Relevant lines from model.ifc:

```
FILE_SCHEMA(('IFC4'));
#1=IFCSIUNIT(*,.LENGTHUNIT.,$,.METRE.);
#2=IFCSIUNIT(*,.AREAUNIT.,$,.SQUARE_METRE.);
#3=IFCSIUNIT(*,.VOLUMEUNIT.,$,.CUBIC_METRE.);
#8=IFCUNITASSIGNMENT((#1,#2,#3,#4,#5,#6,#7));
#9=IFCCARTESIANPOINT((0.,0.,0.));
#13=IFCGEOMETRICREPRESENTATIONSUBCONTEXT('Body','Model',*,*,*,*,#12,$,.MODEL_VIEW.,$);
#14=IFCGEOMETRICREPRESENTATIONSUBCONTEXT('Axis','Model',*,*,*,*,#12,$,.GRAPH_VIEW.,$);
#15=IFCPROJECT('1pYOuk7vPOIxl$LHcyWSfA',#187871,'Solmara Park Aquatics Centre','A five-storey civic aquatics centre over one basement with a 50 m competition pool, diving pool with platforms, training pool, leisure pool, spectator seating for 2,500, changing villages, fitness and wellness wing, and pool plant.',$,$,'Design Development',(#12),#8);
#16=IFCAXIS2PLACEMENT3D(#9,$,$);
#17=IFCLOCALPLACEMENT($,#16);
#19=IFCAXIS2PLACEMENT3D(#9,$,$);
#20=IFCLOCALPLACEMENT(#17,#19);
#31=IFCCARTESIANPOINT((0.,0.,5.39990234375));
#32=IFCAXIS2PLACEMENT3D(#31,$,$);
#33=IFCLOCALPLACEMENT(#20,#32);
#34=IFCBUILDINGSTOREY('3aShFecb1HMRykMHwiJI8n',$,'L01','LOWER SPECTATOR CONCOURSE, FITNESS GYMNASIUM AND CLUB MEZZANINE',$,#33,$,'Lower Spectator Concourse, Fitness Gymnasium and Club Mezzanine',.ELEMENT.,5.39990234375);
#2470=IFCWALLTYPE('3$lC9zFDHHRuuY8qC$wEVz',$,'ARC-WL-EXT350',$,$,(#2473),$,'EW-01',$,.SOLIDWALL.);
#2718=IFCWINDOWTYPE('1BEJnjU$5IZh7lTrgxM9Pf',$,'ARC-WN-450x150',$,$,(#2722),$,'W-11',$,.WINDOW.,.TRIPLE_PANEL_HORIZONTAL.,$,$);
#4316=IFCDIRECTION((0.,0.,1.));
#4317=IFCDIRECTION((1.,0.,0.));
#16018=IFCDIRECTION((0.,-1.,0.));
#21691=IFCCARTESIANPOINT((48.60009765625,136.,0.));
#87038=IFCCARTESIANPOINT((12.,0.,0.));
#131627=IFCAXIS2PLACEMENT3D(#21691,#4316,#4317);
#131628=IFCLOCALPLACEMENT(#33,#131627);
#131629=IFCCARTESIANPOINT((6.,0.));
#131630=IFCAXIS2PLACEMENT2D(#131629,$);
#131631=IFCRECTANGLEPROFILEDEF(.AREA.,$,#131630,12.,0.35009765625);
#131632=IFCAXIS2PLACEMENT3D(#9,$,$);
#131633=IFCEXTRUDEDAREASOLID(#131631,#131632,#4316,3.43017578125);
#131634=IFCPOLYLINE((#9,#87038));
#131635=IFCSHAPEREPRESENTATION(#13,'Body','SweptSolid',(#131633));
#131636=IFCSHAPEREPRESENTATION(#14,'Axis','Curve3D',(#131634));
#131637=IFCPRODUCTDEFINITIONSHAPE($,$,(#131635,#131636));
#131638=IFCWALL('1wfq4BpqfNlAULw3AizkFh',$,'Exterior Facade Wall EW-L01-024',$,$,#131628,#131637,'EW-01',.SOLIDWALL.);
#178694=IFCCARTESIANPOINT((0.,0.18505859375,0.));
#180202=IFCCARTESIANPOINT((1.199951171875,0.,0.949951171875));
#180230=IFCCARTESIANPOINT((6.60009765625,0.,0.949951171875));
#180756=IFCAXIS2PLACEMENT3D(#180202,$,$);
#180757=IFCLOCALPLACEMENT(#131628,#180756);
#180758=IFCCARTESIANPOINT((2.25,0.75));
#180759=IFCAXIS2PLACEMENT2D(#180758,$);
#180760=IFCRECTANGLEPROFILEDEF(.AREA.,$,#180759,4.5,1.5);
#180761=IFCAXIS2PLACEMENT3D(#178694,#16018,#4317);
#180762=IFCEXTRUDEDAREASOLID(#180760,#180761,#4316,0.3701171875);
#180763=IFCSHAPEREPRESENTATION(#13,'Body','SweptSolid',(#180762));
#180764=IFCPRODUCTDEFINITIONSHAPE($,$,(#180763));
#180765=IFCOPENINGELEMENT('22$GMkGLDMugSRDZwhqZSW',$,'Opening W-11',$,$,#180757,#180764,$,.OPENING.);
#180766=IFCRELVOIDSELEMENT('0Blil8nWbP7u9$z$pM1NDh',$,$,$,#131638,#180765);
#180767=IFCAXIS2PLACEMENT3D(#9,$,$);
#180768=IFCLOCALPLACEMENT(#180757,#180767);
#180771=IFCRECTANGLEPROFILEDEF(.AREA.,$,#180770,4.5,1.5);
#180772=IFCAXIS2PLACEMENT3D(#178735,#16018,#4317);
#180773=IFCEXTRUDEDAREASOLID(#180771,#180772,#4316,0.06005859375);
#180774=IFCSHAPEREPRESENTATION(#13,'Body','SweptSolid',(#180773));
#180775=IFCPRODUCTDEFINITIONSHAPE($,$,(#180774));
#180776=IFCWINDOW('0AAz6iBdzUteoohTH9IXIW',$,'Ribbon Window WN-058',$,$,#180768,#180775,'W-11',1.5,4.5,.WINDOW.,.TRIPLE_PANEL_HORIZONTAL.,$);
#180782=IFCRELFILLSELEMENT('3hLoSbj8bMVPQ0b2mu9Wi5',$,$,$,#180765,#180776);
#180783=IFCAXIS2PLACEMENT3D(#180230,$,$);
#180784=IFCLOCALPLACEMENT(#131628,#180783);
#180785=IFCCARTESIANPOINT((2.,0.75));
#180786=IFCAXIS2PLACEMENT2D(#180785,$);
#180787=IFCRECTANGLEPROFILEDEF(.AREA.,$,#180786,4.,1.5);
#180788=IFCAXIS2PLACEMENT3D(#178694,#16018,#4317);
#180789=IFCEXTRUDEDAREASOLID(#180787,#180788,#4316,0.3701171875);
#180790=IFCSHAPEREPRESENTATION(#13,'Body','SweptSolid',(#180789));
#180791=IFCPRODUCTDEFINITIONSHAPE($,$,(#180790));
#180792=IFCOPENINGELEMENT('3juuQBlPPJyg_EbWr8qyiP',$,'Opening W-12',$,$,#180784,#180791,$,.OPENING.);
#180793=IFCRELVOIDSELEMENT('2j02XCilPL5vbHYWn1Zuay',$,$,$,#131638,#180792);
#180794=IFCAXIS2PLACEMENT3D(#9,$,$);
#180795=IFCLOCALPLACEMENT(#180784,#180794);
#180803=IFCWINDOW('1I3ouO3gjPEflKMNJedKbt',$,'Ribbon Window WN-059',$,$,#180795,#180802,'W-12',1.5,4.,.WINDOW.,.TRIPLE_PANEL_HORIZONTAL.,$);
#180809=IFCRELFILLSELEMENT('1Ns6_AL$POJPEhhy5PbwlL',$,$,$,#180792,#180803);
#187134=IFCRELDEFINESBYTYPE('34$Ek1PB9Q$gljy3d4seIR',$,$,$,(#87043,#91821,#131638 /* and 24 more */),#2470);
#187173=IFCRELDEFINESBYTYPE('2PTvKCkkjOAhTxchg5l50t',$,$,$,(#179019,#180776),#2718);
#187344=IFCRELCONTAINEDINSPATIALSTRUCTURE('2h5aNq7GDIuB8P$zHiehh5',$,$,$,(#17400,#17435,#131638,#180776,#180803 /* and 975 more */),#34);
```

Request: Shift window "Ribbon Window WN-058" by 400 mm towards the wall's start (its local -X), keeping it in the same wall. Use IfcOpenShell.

```python
import ifcopenshell
import ifcopenshell.api.geometry
import ifcopenshell.util.placement
import ifcopenshell.util.unit

model = ifcopenshell.open("model.ifc")
unit_scale = ifcopenshell.util.unit.calculate_unit_scale(model)

window = model.by_guid("0AAz6iBdzUteoohTH9IXIW")
opening = window.FillsVoids[0].RelatingOpeningElement
wall = opening.VoidsElements[0].RelatingBuildingElement

wall_matrix = ifcopenshell.util.placement.get_local_placement(wall.ObjectPlacement)
shift = wall_matrix[:3, 0] * -0.4 / unit_scale
before = ifcopenshell.util.placement.get_local_placement(window.ObjectPlacement)[:3, 3].copy()

# The window is placed relative to its opening, so it follows when the opening moves.
matrix = ifcopenshell.util.placement.get_local_placement(opening.ObjectPlacement)
matrix[:3, 3] += shift
ifcopenshell.api.geometry.edit_object_placement(
    model, product=opening, matrix=matrix, is_si=False, should_transform_children=True
)

after = ifcopenshell.util.placement.get_local_placement(window.ObjectPlacement)[:3, 3]
print("window moved by", (after - before).round(3) + 0.0)

model.write("model-out.ifc")
```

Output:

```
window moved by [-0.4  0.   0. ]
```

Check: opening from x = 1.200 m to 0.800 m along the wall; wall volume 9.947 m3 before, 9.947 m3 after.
